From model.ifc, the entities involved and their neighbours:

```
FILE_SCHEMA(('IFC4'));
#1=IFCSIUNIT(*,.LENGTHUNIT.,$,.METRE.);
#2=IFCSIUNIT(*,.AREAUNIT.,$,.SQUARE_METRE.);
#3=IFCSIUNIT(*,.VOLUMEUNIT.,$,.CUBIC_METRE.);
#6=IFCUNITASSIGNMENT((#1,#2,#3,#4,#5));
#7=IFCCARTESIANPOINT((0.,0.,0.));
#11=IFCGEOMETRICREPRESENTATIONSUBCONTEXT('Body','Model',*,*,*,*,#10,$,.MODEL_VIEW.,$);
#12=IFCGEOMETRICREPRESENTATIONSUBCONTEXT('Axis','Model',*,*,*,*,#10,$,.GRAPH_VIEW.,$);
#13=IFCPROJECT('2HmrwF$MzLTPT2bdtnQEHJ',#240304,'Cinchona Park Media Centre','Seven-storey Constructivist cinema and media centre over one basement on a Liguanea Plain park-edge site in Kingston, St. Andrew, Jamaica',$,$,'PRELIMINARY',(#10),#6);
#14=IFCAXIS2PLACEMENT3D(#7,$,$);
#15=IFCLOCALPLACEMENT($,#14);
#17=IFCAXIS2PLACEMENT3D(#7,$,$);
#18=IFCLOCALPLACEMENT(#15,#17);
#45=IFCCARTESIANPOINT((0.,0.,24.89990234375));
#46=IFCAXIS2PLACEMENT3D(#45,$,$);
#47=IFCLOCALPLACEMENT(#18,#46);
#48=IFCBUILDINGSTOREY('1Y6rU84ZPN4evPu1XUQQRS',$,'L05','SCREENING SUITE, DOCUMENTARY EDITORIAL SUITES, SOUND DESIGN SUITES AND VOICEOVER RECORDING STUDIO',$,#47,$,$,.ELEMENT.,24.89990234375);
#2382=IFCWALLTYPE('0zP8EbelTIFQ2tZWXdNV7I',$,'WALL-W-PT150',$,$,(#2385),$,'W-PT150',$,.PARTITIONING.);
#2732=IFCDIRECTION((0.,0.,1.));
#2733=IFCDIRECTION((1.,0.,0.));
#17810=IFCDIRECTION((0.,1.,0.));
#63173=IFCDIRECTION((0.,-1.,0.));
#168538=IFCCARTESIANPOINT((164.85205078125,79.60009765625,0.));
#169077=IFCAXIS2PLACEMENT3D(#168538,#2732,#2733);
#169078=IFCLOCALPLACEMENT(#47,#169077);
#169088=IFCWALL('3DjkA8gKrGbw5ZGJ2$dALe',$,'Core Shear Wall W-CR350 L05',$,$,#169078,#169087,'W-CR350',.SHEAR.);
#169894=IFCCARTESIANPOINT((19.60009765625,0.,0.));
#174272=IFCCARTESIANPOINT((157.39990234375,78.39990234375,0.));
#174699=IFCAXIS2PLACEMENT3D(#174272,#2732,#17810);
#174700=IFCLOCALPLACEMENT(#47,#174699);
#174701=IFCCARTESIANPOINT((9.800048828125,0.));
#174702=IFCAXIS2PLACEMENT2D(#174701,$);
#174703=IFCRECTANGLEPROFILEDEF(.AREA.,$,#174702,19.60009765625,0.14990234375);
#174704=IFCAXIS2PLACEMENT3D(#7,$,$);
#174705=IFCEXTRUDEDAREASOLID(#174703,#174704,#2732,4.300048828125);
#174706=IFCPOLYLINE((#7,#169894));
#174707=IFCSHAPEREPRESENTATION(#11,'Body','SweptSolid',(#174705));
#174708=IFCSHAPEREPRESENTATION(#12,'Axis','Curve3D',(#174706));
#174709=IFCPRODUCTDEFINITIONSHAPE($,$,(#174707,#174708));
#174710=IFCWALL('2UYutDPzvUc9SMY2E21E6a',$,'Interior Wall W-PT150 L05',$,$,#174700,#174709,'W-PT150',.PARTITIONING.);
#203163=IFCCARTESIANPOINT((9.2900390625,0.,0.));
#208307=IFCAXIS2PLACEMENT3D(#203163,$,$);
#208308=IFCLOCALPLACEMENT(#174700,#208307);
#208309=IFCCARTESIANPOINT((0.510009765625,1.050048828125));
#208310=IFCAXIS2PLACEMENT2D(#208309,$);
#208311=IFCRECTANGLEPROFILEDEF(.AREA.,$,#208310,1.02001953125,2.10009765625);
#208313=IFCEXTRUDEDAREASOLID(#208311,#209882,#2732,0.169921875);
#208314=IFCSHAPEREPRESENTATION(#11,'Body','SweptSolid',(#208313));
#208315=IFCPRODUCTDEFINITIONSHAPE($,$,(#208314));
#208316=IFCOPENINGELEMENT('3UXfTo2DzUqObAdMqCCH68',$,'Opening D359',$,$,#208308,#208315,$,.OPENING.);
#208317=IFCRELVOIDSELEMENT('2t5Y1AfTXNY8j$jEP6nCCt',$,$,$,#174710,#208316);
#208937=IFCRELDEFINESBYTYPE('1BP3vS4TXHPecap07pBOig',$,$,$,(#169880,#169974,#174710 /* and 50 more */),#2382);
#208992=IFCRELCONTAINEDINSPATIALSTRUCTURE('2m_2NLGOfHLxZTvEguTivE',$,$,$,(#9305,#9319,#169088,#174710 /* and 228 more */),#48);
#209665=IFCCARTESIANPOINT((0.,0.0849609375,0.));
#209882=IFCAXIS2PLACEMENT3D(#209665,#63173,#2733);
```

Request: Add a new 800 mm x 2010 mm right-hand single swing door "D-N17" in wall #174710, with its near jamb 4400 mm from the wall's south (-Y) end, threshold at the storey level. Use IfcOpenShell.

```python
import numpy as np
import ifcopenshell
import ifcopenshell.api.feature
import ifcopenshell.api.geometry
import ifcopenshell.api.root
import ifcopenshell.api.spatial
import ifcopenshell.geom
import ifcopenshell.util.element
import ifcopenshell.util.placement
import ifcopenshell.util.representation
import ifcopenshell.util.shape
import ifcopenshell.util.unit

model = ifcopenshell.open("model.ifc")
unit_scale = ifcopenshell.util.unit.calculate_unit_scale(model)
settings = ifcopenshell.geom.settings()


def volume(element):
    """Net volume in cubic metres, openings subtracted."""
    shape = ifcopenshell.geom.create_shape(settings, element)
    return ifcopenshell.util.shape.get_volume(shape.geometry)


wall = model.by_guid("2UYutDPzvUc9SMY2E21E6a")
storey = ifcopenshell.util.element.get_container(wall, ifc_class="IfcBuildingStorey")
context = ifcopenshell.util.representation.get_context(model, "Model", "Body", "MODEL_VIEW")
before = volume(wall)

width, height, from_end, sill = 0.8, 2.01, 4.4, 0.0  # metres

# The wall runs along its own X axis, and the end named is its -X end.
wall_shape = ifcopenshell.geom.create_shape(settings, wall)
x, y, z = ifcopenshell.util.shape.get_vertices(wall_shape.geometry).T
start = x.min() + from_end
face, thickness = float(y.min()), float(y.max() - y.min())
wall_matrix = ifcopenshell.util.placement.get_local_placement(wall.ObjectPlacement)
level = ifcopenshell.util.placement.get_local_placement(storey.ObjectPlacement)[2, 3]


def in_wall(x, y):
    """Placement at x, y metres in the wall's axes, at sill height."""
    matrix = wall_matrix.copy()
    matrix[:, 3] = wall_matrix @ np.array([x / unit_scale, y / unit_scale, 0.0, 1.0])
    matrix[2, 3] = level + sill / unit_scale
    return matrix


# Opening: a box that overshoots both wall faces by 50 mm.
opening = ifcopenshell.api.root.create_entity(model, ifc_class="IfcOpeningElement", predefined_type="OPENING")
box = ifcopenshell.api.geometry.add_wall_representation(
    model, context=context, length=width, height=height, thickness=thickness + 0.1
)
ifcopenshell.api.geometry.assign_representation(model, product=opening, representation=box)
ifcopenshell.api.geometry.edit_object_placement(model, product=opening, matrix=in_wall(start, face - 0.05), is_si=False)
ifcopenshell.api.feature.add_feature(model, feature=opening, element=wall)

door = ifcopenshell.api.root.create_entity(model, ifc_class="IfcDoor", name="D-N17", predefined_type="DOOR")
door.OverallWidth, door.OverallHeight = width / unit_scale, height / unit_scale
door.OperationType = "SINGLE_SWING_RIGHT"
body = ifcopenshell.api.geometry.add_door_representation(
    model,
    context=context,
    overall_width=door.OverallWidth,
    overall_height=door.OverallHeight,
    operation_type="SINGLE_SWING_RIGHT",
    lining_properties={"LiningDepth": thickness / unit_scale, "ThresholdDepth": thickness / unit_scale},
)
ifcopenshell.api.geometry.assign_representation(model, product=door, representation=body)
ifcopenshell.api.spatial.assign_container(model, products=[door], relating_structure=storey)
ifcopenshell.api.feature.add_filling(model, opening=opening, element=door)

# The lining spans the wall, so the door starts at the wall face.
ifcopenshell.api.geometry.edit_object_placement(model, product=door, matrix=in_wall(start, face), is_si=False)

after = volume(wall)

print(f"wall volume {before:.3f} -> {after:.3f} m3")

model.write("model_v2.ifc")
```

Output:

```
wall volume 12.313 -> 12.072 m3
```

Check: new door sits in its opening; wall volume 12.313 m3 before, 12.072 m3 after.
